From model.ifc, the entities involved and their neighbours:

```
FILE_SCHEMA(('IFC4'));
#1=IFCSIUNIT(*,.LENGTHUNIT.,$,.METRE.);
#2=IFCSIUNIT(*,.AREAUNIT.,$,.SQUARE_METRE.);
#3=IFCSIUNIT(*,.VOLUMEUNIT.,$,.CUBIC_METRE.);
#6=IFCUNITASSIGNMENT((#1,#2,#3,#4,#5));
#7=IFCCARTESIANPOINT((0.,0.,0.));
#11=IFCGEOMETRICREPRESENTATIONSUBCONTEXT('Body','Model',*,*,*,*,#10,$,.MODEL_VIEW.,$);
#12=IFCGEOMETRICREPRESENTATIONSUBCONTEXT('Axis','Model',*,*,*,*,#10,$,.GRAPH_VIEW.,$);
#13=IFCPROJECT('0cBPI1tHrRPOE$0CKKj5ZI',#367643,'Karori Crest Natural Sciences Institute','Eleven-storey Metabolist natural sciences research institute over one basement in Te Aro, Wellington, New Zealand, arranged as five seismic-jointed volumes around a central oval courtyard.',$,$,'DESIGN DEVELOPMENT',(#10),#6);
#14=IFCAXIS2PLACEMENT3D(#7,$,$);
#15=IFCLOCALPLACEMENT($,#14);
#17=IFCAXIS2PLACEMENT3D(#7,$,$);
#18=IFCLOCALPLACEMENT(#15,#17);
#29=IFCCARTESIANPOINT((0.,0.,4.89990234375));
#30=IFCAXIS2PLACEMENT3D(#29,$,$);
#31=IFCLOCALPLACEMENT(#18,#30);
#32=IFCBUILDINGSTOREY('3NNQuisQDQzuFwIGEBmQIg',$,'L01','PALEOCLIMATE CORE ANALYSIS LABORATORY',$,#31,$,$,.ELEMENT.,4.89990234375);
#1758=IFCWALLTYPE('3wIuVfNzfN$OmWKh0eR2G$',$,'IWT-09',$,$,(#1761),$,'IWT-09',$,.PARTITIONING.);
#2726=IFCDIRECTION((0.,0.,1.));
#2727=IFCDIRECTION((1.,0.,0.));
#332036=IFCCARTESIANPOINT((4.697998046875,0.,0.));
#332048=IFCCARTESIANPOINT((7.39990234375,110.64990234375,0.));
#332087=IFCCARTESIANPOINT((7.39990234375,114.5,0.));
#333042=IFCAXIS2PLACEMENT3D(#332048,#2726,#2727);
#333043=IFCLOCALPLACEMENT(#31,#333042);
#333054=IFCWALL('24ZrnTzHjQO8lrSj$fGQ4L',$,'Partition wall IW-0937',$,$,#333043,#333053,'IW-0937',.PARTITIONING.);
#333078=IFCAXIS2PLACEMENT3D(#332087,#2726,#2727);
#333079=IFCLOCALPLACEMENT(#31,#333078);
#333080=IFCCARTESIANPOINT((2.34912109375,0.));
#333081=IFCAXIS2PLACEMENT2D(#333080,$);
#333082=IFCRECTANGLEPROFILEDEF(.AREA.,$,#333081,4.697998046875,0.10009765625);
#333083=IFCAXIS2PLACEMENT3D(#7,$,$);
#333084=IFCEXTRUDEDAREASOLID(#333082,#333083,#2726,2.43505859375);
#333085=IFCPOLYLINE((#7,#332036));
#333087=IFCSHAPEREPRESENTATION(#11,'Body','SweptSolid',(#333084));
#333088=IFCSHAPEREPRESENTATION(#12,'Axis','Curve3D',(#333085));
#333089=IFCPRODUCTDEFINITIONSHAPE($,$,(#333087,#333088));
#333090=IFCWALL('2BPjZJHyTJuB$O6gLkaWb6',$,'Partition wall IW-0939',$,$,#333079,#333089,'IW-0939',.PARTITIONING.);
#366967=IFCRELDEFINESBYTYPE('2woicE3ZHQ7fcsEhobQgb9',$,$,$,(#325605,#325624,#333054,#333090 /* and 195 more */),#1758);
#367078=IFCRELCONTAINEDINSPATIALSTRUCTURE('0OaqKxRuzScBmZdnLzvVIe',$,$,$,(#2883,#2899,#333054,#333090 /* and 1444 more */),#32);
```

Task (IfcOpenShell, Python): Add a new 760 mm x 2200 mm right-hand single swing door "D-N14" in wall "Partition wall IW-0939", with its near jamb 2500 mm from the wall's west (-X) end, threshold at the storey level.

```python
import numpy as np
import ifcopenshell
import ifcopenshell.api.feature
import ifcopenshell.api.geometry
import ifcopenshell.api.root
import ifcopenshell.api.spatial
import ifcopenshell.geom
import ifcopenshell.util.element
import ifcopenshell.util.placement
import ifcopenshell.util.representation
import ifcopenshell.util.shape
import ifcopenshell.util.unit

model = ifcopenshell.open("model.ifc")
unit_scale = ifcopenshell.util.unit.calculate_unit_scale(model)
settings = ifcopenshell.geom.settings()


def volume(element):
    """Net volume in cubic metres, openings subtracted."""
    shape = ifcopenshell.geom.create_shape(settings, element)
    return ifcopenshell.util.shape.get_volume(shape.geometry)


wall = model.by_id(333090)
storey = ifcopenshell.util.element.get_container(wall, ifc_class="IfcBuildingStorey")
context = ifcopenshell.util.representation.get_context(model, "Model", "Body", "MODEL_VIEW")
before = volume(wall)

width, height, from_end, sill = 0.76, 2.2, 2.5, 0.0  # metres

# The wall runs along its own X axis, and the end named is its -X end.
wall_shape = ifcopenshell.geom.create_shape(settings, wall)
x, y, z = ifcopenshell.util.shape.get_vertices(wall_shape.geometry).T
start = x.min() + from_end
face, thickness = float(y.min()), float(y.max() - y.min())
wall_matrix = ifcopenshell.util.placement.get_local_placement(wall.ObjectPlacement)
level = ifcopenshell.util.placement.get_local_placement(storey.ObjectPlacement)[2, 3]


def in_wall(x, y):
    """Placement at x, y metres in the wall's axes, at sill height."""
    matrix = wall_matrix.copy()
    matrix[:, 3] = wall_matrix @ np.array([x / unit_scale, y / unit_scale, 0.0, 1.0])
    matrix[2, 3] = level + sill / unit_scale
    return matrix


# Opening: a box that overshoots both wall faces by 50 mm.
opening = ifcopenshell.api.root.create_entity(model, ifc_class="IfcOpeningElement", predefined_type="OPENING")
box = ifcopenshell.api.geometry.add_wall_representation(
    model, context=context, length=width, height=height, thickness=thickness + 0.1
)
ifcopenshell.api.geometry.assign_representation(model, product=opening, representation=box)
ifcopenshell.api.geometry.edit_object_placement(model, product=opening, matrix=in_wall(start, face - 0.05), is_si=False)
ifcopenshell.api.feature.add_feature(model, feature=opening, element=wall)

door = ifcopenshell.api.root.create_entity(model, ifc_class="IfcDoor", name="D-N14", predefined_type="DOOR")
door.OverallWidth, door.OverallHeight = width / unit_scale, height / unit_scale
door.OperationType = "SINGLE_SWING_RIGHT"
body = ifcopenshell.api.geometry.add_door_representation(
    model,
    context=context,
    overall_width=door.OverallWidth,
    overall_height=door.OverallHeight,
    operation_type="SINGLE_SWING_RIGHT",
    lining_properties={"LiningDepth": thickness / unit_scale, "ThresholdDepth": thickness / unit_scale},
)
ifcopenshell.api.geometry.assign_representation(model, product=door, representation=body)
ifcopenshell.api.spatial.assign_container(model, products=[door], relating_structure=storey)
ifcopenshell.api.feature.add_filling(model, opening=opening, element=door)

# The lining spans the wall, so the door starts at the wall face.
ifcopenshell.api.geometry.edit_object_placement(model, product=door, matrix=in_wall(start, face), is_si=False)

after = volume(wall)

print(f"wall volume {before:.3f} -> {after:.3f} m3")

model.write("model-out.ifc")
```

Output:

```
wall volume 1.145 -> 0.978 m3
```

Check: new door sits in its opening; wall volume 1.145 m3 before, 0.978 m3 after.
